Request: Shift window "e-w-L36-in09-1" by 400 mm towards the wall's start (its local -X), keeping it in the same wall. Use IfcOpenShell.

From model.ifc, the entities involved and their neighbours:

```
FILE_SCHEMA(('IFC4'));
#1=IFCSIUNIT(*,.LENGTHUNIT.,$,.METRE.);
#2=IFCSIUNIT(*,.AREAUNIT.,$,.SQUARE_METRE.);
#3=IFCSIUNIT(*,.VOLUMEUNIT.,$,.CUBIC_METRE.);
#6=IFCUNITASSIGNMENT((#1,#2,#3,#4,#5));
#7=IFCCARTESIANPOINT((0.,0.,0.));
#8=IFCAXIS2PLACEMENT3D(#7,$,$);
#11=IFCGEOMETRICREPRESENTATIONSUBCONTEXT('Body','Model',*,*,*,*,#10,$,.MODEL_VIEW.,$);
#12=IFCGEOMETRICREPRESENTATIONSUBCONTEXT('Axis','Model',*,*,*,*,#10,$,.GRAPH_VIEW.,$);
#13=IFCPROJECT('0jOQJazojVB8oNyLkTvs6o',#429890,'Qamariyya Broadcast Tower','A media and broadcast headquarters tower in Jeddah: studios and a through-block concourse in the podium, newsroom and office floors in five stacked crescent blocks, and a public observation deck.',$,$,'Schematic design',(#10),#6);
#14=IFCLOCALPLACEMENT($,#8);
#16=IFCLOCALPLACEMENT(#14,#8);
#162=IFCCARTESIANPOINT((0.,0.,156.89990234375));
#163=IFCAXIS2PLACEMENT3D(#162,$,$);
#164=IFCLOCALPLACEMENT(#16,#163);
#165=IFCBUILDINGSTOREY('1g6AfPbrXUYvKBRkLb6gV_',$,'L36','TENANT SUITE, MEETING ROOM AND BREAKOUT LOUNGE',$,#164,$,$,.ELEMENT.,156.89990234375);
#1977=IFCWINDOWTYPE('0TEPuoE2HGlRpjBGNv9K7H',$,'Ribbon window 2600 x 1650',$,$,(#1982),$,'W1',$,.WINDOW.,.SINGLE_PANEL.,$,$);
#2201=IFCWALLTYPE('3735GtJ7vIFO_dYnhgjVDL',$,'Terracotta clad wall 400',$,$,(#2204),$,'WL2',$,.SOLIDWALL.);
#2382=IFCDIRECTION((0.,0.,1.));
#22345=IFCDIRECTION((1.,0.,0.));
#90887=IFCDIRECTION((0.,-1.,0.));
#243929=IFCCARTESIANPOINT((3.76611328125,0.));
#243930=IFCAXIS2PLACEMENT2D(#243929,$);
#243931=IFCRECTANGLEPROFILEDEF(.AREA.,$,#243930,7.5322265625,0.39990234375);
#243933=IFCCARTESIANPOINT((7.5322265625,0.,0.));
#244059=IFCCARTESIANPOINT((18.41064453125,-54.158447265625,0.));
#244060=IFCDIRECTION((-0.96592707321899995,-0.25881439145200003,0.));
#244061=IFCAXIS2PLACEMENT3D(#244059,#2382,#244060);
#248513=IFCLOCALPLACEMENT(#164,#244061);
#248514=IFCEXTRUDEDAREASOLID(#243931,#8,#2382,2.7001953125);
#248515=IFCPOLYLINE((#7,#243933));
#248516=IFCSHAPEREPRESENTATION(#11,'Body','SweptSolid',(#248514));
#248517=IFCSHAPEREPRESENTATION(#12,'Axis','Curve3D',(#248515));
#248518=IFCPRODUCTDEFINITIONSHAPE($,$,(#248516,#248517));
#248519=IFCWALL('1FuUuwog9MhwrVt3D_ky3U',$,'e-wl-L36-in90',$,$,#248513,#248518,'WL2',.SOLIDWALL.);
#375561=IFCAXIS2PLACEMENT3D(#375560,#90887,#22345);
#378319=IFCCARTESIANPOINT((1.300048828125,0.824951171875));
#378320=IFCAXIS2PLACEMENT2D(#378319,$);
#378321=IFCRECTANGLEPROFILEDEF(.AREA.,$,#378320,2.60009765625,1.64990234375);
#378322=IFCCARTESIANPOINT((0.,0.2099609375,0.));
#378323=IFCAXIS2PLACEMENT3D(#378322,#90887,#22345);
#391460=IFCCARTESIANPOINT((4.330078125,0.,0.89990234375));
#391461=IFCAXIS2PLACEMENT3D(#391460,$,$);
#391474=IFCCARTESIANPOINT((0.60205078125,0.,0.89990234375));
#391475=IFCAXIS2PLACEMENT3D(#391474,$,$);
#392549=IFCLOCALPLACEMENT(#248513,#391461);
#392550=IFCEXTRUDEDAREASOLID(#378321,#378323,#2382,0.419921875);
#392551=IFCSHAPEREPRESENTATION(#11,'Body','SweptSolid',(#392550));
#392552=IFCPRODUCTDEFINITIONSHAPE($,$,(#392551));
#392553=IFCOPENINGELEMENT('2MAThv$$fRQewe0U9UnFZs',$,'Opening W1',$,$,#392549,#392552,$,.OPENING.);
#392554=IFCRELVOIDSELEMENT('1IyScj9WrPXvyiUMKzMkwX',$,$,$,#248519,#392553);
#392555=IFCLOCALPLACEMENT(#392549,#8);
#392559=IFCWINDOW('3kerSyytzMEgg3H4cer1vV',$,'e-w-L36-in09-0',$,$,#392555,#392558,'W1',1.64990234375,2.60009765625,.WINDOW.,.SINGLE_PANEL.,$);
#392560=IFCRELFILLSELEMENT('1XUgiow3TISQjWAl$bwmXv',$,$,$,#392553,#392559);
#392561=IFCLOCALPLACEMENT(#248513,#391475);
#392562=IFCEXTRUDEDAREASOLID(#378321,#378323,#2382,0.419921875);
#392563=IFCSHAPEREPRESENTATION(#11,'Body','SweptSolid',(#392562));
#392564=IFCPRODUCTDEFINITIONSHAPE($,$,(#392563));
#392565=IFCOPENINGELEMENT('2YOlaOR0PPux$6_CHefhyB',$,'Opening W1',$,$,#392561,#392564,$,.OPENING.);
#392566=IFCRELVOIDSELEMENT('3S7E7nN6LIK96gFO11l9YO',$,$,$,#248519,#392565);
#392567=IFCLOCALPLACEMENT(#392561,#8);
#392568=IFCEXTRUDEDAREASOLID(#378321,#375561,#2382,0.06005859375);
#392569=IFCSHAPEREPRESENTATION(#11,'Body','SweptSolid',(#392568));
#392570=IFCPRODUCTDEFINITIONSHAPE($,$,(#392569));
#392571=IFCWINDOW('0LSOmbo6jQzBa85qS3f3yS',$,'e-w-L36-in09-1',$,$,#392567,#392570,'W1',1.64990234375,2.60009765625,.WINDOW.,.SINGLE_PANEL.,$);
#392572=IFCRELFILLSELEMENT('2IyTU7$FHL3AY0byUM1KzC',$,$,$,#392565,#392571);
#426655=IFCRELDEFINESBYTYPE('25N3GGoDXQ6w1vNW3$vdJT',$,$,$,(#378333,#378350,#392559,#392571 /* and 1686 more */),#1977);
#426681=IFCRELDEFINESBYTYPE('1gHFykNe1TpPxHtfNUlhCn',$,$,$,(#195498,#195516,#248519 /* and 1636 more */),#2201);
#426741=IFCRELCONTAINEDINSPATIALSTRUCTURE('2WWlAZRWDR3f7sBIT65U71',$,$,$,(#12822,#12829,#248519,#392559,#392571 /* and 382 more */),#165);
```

```python
import ifcopenshell
import ifcopenshell.api.geometry
import ifcopenshell.util.placement
import ifcopenshell.util.unit

model = ifcopenshell.open("model.ifc")
unit_scale = ifcopenshell.util.unit.calculate_unit_scale(model)

window = model.by_guid("0LSOmbo6jQzBa85qS3f3yS")
opening = window.FillsVoids[0].RelatingOpeningElement
wall = opening.VoidsElements[0].RelatingBuildingElement

wall_matrix = ifcopenshell.util.placement.get_local_placement(wall.ObjectPlacement)
shift = wall_matrix[:3, 0] * -0.4 / unit_scale
before = ifcopenshell.util.placement.get_local_placement(window.ObjectPlacement)[:3, 3].copy()

# The window is placed relative to its opening, so it follows when the opening moves.
matrix = ifcopenshell.util.placement.get_local_placement(opening.ObjectPlacement)
matrix[:3, 3] += shift
ifcopenshell.api.geometry.edit_object_placement(
    model, product=opening, matrix=matrix, is_si=False, should_transform_children=True
)

after = ifcopenshell.util.placement.get_local_placement(window.ObjectPlacement)[:3, 3]
print("window moved by", (after - before).round(3) + 0.0)

model.write("model_updated.ifc")
```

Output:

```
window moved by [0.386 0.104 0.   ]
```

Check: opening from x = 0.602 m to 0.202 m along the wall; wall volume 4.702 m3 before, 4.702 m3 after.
